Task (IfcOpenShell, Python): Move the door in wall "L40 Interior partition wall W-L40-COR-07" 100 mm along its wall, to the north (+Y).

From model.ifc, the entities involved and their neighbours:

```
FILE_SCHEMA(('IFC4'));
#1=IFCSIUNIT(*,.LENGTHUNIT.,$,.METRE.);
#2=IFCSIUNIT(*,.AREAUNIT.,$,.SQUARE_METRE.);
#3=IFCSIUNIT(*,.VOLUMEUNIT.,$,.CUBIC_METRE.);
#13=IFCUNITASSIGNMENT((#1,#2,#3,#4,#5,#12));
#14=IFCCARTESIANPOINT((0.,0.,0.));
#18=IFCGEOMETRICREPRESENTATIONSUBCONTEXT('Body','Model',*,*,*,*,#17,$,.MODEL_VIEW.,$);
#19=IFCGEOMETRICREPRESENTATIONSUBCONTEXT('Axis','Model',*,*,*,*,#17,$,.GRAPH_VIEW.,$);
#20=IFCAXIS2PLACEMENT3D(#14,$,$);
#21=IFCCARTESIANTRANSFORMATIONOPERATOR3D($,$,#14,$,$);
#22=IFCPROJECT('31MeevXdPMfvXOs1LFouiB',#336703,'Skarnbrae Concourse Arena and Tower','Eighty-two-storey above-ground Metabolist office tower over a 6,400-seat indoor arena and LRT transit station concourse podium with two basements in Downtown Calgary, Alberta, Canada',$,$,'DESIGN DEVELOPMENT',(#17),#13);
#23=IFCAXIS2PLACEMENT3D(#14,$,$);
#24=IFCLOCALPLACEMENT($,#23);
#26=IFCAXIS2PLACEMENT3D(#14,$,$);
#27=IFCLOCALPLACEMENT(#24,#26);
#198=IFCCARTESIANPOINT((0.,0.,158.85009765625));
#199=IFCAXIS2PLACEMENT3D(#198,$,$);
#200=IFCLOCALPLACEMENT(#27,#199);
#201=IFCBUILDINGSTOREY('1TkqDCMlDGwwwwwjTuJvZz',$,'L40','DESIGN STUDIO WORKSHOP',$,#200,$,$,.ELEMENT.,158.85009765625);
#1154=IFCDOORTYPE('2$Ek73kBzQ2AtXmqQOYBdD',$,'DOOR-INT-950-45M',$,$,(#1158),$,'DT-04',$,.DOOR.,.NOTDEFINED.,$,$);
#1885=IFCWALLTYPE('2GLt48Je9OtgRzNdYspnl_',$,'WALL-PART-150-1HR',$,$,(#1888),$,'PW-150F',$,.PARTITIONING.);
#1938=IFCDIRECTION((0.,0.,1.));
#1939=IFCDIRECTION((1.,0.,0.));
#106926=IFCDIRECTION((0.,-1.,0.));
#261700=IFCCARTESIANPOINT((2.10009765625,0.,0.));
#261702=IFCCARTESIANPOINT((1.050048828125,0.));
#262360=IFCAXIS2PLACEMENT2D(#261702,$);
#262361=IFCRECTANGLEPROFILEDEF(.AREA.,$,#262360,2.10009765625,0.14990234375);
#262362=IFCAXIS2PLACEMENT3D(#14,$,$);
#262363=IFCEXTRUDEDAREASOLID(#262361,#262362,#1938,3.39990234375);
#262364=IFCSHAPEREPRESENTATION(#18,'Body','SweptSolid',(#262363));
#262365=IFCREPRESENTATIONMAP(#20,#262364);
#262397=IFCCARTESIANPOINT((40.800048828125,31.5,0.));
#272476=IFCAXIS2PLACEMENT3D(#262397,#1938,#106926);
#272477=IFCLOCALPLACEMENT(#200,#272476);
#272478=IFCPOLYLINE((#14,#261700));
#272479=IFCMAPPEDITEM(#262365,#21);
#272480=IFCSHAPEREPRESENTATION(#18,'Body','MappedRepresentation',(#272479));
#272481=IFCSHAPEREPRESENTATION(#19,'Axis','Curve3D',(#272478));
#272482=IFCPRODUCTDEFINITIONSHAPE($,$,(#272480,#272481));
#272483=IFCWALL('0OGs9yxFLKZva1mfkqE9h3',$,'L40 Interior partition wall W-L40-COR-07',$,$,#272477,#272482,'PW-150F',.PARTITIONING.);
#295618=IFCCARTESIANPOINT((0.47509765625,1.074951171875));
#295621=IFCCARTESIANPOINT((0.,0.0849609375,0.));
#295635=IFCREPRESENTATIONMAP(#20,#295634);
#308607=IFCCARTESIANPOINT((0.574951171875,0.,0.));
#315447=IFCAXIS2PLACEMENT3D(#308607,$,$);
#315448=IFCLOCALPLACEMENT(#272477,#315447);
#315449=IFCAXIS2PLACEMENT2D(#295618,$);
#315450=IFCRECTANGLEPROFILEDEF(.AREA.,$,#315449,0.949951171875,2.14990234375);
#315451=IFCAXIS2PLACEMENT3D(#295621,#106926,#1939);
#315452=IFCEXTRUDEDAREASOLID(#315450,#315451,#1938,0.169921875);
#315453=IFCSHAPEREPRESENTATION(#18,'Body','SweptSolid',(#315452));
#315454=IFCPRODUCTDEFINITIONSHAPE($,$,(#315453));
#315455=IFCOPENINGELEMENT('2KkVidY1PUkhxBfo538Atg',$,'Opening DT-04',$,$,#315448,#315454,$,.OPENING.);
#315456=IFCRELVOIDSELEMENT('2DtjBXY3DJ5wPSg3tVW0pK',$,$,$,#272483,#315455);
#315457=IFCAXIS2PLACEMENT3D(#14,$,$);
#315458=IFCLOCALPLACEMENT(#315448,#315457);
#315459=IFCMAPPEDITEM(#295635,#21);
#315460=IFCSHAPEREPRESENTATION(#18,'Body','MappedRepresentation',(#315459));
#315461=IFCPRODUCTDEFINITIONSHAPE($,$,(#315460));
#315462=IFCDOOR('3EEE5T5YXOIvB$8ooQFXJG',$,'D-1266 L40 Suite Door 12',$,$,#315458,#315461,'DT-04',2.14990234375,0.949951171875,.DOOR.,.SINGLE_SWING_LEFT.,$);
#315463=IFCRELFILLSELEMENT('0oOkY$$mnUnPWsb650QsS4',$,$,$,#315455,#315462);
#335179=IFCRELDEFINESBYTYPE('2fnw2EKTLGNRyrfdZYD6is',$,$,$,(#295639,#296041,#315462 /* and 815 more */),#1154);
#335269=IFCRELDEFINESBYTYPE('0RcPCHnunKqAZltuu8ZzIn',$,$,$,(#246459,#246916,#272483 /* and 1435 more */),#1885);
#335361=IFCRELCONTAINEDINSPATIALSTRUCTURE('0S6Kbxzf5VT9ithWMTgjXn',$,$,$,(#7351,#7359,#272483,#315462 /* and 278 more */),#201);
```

```python
import ifcopenshell
import ifcopenshell.api.geometry
import ifcopenshell.util.placement

model = ifcopenshell.open("model.ifc")

door = model.by_guid("3EEE5T5YXOIvB$8ooQFXJG")
opening = door.FillsVoids[0].RelatingOpeningElement
wall = opening.VoidsElements[0].RelatingBuildingElement

wall_matrix = ifcopenshell.util.placement.get_local_placement(wall.ObjectPlacement)
shift = wall_matrix[:3, 0] * -0.1
before = ifcopenshell.util.placement.get_local_placement(door.ObjectPlacement)[:3, 3].copy()

# The door is placed relative to its opening, so it follows when the opening moves.
matrix = ifcopenshell.util.placement.get_local_placement(opening.ObjectPlacement)
matrix[:3, 3] += shift
ifcopenshell.api.geometry.edit_object_placement(
    model, product=opening, matrix=matrix, is_si=False, should_transform_children=True
)

after = ifcopenshell.util.placement.get_local_placement(door.ObjectPlacement)[:3, 3]
print("door moved by", (after - before).round(3) + 0.0)

model.write("model-out.ifc")
```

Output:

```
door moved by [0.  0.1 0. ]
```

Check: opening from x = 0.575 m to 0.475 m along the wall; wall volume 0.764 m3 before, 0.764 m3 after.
